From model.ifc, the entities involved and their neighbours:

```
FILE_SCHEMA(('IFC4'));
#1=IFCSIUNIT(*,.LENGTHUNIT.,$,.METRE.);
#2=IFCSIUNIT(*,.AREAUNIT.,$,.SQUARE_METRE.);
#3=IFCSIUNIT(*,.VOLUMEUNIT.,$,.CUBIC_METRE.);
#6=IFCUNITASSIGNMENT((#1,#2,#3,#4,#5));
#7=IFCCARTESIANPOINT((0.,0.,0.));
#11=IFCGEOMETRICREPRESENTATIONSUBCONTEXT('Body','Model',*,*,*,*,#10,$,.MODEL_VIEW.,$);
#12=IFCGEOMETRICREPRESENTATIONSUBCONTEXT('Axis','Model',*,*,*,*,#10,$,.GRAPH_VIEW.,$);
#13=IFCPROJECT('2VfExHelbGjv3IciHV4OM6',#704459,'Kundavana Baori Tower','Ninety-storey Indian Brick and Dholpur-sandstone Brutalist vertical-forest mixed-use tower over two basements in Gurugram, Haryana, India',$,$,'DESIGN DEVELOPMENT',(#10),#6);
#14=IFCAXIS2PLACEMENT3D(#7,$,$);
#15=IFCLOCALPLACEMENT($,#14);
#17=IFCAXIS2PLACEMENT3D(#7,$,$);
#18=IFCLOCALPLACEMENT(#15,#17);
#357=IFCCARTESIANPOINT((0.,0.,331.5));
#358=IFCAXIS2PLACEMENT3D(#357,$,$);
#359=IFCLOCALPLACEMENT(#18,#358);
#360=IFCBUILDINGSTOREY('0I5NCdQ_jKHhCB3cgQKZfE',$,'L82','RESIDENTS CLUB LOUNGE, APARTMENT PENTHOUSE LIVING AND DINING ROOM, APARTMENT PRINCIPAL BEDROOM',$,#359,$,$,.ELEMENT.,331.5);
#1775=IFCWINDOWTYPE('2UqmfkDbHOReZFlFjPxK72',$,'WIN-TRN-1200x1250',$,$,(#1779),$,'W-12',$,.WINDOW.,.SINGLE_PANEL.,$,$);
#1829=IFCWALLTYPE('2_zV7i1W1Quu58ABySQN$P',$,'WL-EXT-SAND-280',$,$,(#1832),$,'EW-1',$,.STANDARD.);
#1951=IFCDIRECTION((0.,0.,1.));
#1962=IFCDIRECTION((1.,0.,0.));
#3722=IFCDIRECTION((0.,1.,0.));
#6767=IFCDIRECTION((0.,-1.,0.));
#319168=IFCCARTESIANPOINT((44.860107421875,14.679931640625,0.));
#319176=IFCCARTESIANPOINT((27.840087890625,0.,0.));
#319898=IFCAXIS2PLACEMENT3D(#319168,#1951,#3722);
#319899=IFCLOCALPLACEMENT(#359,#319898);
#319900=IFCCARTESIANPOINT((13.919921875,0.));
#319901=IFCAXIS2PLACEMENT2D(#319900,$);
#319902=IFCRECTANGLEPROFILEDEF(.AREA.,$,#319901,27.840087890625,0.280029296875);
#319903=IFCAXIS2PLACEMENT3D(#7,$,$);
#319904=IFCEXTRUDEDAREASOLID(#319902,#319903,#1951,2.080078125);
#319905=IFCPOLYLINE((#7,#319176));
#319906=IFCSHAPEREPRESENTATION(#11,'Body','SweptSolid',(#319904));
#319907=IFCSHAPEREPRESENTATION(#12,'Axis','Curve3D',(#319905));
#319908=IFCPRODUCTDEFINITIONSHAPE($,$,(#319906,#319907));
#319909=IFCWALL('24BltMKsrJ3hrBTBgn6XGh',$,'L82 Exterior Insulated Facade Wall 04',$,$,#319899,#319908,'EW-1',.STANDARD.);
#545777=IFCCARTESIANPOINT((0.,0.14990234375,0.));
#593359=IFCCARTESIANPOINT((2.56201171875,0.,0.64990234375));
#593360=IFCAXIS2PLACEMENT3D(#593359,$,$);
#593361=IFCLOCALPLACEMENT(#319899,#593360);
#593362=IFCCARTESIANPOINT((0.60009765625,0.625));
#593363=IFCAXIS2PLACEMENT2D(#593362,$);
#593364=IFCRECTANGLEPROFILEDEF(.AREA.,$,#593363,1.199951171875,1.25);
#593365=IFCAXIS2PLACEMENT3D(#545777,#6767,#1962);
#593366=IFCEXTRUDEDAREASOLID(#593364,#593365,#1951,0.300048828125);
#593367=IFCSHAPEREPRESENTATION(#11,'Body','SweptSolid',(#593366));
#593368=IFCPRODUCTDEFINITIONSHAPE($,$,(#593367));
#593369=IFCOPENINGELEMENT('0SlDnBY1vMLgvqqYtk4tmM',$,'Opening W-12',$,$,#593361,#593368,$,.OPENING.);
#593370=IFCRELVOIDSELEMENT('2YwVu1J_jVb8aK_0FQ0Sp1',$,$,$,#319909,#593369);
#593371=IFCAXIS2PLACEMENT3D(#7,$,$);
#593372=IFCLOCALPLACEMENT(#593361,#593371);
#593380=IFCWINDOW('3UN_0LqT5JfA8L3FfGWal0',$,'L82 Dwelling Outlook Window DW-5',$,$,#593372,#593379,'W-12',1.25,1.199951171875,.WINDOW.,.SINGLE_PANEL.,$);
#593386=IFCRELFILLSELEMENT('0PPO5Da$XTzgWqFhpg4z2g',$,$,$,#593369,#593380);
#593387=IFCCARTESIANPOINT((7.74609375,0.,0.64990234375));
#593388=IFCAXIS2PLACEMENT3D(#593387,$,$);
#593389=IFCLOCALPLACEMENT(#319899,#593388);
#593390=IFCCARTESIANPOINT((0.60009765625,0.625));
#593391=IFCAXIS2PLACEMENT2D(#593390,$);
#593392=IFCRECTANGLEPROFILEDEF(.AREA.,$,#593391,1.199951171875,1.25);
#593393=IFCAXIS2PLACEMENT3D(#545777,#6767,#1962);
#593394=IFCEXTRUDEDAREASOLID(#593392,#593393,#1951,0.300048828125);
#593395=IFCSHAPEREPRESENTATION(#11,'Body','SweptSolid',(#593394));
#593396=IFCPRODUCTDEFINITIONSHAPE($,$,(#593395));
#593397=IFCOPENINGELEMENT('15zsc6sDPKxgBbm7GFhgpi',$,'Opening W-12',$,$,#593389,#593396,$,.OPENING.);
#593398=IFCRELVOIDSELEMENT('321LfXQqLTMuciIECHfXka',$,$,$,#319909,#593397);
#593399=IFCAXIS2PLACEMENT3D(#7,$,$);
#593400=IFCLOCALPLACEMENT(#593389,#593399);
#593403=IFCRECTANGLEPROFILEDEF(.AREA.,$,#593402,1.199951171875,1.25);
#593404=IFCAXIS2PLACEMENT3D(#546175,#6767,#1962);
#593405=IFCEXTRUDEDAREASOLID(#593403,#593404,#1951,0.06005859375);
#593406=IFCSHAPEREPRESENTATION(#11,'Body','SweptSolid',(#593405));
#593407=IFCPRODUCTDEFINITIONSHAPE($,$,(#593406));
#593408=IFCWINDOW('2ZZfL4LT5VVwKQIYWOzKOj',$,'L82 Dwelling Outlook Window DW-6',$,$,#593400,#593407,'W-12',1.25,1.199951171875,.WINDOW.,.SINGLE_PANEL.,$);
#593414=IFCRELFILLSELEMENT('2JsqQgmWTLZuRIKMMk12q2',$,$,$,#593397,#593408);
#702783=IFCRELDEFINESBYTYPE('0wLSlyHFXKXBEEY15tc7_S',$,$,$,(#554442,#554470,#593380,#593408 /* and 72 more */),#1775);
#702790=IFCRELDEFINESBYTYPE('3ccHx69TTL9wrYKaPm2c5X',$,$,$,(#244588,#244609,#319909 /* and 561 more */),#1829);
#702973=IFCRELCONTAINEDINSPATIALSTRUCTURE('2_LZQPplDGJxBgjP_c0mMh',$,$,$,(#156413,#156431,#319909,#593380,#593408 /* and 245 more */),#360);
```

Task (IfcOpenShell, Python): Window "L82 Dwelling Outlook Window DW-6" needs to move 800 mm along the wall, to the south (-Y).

```python
import ifcopenshell
import ifcopenshell.api.geometry
import ifcopenshell.util.placement
import ifcopenshell.util.unit

model = ifcopenshell.open("model.ifc")
unit_scale = ifcopenshell.util.unit.calculate_unit_scale(model)

window = model.by_guid("2ZZfL4LT5VVwKQIYWOzKOj")
opening = window.FillsVoids[0].RelatingOpeningElement
wall = opening.VoidsElements[0].RelatingBuildingElement

wall_matrix = ifcopenshell.util.placement.get_local_placement(wall.ObjectPlacement)
shift = wall_matrix[:3, 0] * -0.8 / unit_scale
before = ifcopenshell.util.placement.get_local_placement(window.ObjectPlacement)[:3, 3].copy()

# The window is placed relative to its opening, so it follows when the opening moves.
matrix = ifcopenshell.util.placement.get_local_placement(opening.ObjectPlacement)
matrix[:3, 3] += shift
ifcopenshell.api.geometry.edit_object_placement(
    model, product=opening, matrix=matrix, is_si=False, should_transform_children=True
)

after = ifcopenshell.util.placement.get_local_placement(window.ObjectPlacement)[:3, 3]
print("window moved by", (after - before).round(3) + 0.0)

model.write("model_edited.ifc")
```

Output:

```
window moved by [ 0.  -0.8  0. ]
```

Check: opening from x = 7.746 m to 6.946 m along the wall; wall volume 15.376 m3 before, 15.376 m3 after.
